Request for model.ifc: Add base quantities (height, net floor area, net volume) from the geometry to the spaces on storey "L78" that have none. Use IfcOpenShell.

First a look at what the model holds.

```python
import ifcopenshell
import ifcopenshell.util.element
import ifcopenshell.util.unit

model = ifcopenshell.open("model.ifc")
print(model.schema)
for unit_type in ("LENGTHUNIT", "AREAUNIT", "VOLUMEUNIT"):
    print(unit_type, ifcopenshell.util.unit.calculate_unit_scale(model, unit_type))
storey = next(s for s in model.by_type("IfcBuildingStorey") if s.Name == "L78")
spaces = [e for e in ifcopenshell.util.element.get_decomposition(storey) if e.is_a("IfcSpace")]
for e in sorted(spaces, key=lambda e: e.id()):
    print(e.id(), e.is_a(), e.Name, list(ifcopenshell.util.element.get_psets(e, qtos_only=True)), sep=" | ")
```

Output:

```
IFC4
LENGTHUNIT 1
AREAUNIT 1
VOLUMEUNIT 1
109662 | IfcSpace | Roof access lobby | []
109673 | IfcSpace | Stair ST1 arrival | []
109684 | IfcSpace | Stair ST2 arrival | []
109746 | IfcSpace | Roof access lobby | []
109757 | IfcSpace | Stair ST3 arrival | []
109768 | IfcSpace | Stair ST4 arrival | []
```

```python
import ifcopenshell
import ifcopenshell.api.pset
import ifcopenshell.geom
import ifcopenshell.util.element
import ifcopenshell.util.shape
import ifcopenshell.util.unit

model = ifcopenshell.open("model.ifc")
unit_scale = ifcopenshell.util.unit.calculate_unit_scale(model)
area_scale = ifcopenshell.util.unit.calculate_unit_scale(model, "AREAUNIT")
volume_scale = ifcopenshell.util.unit.calculate_unit_scale(model, "VOLUMEUNIT")
settings = ifcopenshell.geom.settings()

storey = next(s for s in model.by_type("IfcBuildingStorey") if s.Name == "L78")
spaces = [e for e in ifcopenshell.util.element.get_decomposition(storey) if e.is_a("IfcSpace")]

for e in sorted(spaces, key=lambda e: e.id()):
    if ifcopenshell.util.element.get_psets(e, qtos_only=True, should_inherit=False):
        continue
    # Geometry comes back in metres, in the element's own axes.
    shape = ifcopenshell.geom.create_shape(settings, e)
    values = {
        "Height": ifcopenshell.util.shape.get_z(shape.geometry) / unit_scale,
        "NetFloorArea": ifcopenshell.util.shape.get_footprint_area(shape.geometry) / area_scale,
        "NetVolume": ifcopenshell.util.shape.get_volume(shape.geometry) / volume_scale,
    }
    qto = ifcopenshell.api.pset.add_qto(model, product=e, name="Qto_SpaceBaseQuantities")
    ifcopenshell.api.pset.edit_qto(model, qto=qto, properties=values)
    print(e.id(), {k: round(v, 3) for k, v in values.items()})

model.write("model_updated.ifc")
```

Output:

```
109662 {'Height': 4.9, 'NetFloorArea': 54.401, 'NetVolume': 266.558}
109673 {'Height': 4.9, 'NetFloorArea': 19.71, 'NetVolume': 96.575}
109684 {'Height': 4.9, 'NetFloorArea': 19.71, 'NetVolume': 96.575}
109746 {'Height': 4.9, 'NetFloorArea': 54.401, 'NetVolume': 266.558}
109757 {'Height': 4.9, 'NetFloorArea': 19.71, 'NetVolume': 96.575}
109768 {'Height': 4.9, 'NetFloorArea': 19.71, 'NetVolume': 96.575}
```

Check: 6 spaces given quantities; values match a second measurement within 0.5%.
